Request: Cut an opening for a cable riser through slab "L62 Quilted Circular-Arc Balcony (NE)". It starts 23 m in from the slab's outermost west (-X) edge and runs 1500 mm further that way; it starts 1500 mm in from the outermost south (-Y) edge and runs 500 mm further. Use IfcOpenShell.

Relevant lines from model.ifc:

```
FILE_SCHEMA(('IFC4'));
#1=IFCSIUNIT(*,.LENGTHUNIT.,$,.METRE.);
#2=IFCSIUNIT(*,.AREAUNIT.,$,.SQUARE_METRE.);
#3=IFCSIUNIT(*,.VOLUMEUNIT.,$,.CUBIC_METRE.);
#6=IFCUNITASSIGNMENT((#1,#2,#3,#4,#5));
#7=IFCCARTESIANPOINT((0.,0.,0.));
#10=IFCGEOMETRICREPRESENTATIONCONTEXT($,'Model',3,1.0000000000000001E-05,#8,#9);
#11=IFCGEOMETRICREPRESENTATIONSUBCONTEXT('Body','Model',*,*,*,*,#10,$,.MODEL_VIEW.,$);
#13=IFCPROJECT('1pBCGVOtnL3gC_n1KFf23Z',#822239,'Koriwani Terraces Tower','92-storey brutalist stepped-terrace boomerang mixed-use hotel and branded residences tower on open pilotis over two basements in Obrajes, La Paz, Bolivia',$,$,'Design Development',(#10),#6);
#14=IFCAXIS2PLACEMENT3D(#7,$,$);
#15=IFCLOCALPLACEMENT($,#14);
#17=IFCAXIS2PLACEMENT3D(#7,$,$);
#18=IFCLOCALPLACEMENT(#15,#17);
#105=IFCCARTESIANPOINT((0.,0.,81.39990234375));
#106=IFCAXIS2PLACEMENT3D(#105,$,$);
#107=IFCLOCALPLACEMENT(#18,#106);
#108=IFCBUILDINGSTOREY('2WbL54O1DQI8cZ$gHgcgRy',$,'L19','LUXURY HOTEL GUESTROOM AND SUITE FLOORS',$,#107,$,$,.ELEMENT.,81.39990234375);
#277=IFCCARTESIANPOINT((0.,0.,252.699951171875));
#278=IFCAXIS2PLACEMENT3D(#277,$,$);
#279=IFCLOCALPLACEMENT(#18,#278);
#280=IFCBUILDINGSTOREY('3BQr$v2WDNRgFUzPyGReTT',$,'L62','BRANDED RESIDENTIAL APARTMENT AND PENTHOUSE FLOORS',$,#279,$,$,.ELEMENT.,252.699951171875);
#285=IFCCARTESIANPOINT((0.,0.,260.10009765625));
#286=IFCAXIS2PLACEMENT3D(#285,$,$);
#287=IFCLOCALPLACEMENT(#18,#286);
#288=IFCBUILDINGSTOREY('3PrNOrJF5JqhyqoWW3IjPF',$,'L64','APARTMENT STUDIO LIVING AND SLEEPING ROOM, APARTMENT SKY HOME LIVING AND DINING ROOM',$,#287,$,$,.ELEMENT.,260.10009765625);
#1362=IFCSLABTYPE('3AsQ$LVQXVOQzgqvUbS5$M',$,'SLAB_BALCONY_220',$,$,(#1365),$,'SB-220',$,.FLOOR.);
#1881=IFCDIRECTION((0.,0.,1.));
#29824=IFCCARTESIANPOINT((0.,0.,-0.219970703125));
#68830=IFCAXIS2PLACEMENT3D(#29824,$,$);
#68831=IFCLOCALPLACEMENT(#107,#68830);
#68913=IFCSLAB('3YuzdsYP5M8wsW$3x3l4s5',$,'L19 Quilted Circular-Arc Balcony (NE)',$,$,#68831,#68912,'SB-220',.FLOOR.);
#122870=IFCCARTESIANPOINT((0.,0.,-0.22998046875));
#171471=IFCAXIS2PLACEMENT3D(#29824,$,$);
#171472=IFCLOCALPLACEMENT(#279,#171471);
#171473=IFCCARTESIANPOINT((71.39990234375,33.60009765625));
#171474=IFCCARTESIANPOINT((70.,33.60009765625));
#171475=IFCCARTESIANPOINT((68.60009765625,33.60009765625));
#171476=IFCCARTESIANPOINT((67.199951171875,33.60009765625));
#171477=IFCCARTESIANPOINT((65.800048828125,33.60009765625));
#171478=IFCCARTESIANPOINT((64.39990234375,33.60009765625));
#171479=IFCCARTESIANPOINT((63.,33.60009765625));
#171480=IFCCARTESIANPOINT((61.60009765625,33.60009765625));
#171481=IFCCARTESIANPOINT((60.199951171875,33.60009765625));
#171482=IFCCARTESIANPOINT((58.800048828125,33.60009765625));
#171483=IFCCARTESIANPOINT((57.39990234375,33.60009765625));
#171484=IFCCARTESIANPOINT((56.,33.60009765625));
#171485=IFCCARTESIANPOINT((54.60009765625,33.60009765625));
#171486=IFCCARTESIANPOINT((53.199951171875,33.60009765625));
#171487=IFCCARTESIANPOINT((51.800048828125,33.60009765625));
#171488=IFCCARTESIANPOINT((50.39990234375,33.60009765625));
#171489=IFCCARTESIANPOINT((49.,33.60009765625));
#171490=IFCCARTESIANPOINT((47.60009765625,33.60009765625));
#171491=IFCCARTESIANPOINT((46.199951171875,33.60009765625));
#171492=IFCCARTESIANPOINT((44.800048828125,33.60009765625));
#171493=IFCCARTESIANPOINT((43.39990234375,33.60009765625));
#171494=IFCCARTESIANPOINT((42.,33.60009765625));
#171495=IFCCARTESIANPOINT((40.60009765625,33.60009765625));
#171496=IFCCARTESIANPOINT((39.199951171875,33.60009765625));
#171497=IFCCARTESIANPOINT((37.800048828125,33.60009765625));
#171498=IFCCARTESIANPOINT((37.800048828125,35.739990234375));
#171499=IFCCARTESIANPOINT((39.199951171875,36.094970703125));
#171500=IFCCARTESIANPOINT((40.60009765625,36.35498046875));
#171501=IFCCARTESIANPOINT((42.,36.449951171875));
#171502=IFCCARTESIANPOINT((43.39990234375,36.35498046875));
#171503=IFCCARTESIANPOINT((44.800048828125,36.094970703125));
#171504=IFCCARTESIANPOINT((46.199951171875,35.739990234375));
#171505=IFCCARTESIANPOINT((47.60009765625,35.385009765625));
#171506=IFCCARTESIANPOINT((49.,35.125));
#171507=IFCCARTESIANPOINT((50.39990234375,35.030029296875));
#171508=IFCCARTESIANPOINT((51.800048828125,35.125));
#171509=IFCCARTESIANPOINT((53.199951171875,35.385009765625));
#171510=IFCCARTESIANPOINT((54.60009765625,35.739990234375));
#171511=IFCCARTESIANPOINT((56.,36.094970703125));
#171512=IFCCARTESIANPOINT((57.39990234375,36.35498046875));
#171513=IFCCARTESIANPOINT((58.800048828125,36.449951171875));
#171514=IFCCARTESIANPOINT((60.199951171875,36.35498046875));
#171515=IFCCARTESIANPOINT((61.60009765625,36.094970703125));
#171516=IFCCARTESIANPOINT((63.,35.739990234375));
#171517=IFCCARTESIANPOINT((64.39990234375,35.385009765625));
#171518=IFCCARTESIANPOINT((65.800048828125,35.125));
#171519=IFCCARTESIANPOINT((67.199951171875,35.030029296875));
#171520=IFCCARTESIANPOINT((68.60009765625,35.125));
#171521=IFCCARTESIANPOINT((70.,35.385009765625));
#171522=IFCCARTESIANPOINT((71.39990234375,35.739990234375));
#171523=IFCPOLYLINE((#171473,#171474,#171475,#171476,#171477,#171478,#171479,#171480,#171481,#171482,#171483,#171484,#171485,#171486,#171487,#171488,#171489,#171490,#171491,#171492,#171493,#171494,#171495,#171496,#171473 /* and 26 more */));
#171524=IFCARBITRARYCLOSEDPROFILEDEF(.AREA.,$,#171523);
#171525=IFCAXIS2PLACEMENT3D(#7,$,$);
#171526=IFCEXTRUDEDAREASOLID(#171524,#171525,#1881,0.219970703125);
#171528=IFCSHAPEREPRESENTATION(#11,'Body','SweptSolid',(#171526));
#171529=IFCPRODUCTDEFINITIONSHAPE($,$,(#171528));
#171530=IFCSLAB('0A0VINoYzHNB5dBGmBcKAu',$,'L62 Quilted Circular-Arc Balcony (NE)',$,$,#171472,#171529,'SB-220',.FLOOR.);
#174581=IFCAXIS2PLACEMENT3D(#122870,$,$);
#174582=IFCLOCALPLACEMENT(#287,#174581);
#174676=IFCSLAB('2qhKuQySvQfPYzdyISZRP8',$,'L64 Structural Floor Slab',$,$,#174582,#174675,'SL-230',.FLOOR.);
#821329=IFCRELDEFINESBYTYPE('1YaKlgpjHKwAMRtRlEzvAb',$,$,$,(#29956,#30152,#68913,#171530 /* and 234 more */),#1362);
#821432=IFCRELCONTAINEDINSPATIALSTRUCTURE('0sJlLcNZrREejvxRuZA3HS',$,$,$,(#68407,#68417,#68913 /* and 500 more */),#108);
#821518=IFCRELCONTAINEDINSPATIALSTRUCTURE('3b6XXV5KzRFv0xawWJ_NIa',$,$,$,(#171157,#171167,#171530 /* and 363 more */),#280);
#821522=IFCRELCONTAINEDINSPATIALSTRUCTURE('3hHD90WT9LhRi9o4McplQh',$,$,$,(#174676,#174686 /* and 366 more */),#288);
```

```python
import numpy as np
import ifcopenshell
import ifcopenshell.api.feature
import ifcopenshell.api.geometry
import ifcopenshell.api.root
import ifcopenshell.geom
import ifcopenshell.util.placement
import ifcopenshell.util.representation
import ifcopenshell.util.shape
import ifcopenshell.util.unit

model = ifcopenshell.open("model.ifc")
unit_scale = ifcopenshell.util.unit.calculate_unit_scale(model)
settings = ifcopenshell.geom.settings()


def volume(element):
    """Net volume in cubic metres, openings subtracted."""
    shape = ifcopenshell.geom.create_shape(settings, element)
    return ifcopenshell.util.shape.get_volume(shape.geometry)


slab = model.by_guid("0A0VINoYzHNB5dBGmBcKAu")
before = volume(slab)

# Extent in the slab's own axes, in metres. The edges named are its -X and -Y sides.
slab_shape = ifcopenshell.geom.create_shape(settings, slab)
vertices = ifcopenshell.util.shape.get_vertices(slab_shape.geometry)
x_min, y_min, bottom = vertices.min(axis=0)
top = vertices[:, 2].max()

opening = ifcopenshell.api.root.create_entity(model, ifc_class="IfcOpeningElement", name="Cable riser opening", predefined_type="OPENING")
context = ifcopenshell.util.representation.get_context(model, "Model", "Body", "MODEL_VIEW")
width, depth = 1.5, 0.5
outline = [(0.0, 0.0), (width, 0.0), (width, depth), (0.0, depth), (0.0, 0.0)]
# Overshoot both faces by 50 mm so the cut is clean.
shape = ifcopenshell.api.geometry.add_slab_representation(
    model, context=context, depth=top - bottom + 0.1, polyline=outline
)
ifcopenshell.api.geometry.assign_representation(model, product=opening, representation=shape)

matrix = ifcopenshell.util.placement.get_local_placement(slab.ObjectPlacement)
matrix[:, 3] = matrix @ np.append(np.array([x_min + 23, y_min + 1.5, bottom - 0.05]) / unit_scale, 1.0)
ifcopenshell.api.geometry.edit_object_placement(model, product=opening, matrix=matrix, is_si=False)
ifcopenshell.api.feature.add_feature(model, feature=opening, element=slab)

after = volume(slab)

print(f"slab volume {before:.3f} -> {after:.3f} m3")

model.write("model_edited.ifc")
```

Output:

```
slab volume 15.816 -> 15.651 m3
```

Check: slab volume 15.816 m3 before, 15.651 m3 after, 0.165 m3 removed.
